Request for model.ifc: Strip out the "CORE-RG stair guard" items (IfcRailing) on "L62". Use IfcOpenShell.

First a look at what the model holds.

```python
import ifcopenshell
import ifcopenshell.util.element

model = ifcopenshell.open("model.ifc")
print(model.schema)
storey = next(s for s in model.by_type("IfcBuildingStorey") if s.Name == "L62")
railings = [e for e in ifcopenshell.util.element.get_decomposition(storey) if e.is_a("IfcRailing")]
seen = {}
for e in railings:
    element_type = ifcopenshell.util.element.get_type(e)
    name = element_type.Name if element_type not in (None, e) else None
    seen[name] = seen.get(name, 0) + 1
for name, count in sorted(seen.items(), key=str):
    print(count, "x", name)
```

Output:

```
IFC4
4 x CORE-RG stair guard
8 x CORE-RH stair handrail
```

```python
import ifcopenshell
import ifcopenshell.api.root
import ifcopenshell.util.element

model = ifcopenshell.open("model.ifc")

storey = next(s for s in model.by_type("IfcBuildingStorey") if s.Name == "L62")
railings = [e for e in ifcopenshell.util.element.get_decomposition(storey) if e.is_a("IfcRailing")]
targets = [e for e in railings if (t := ifcopenshell.util.element.get_type(e)) not in (None, e) and t.Name == "CORE-RG stair guard"]

for e in targets:
    ifcopenshell.api.root.remove_product(model, product=e)
print(len(targets), "removed")

model.write("model_updated.ifc")
```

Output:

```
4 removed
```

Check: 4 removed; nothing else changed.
